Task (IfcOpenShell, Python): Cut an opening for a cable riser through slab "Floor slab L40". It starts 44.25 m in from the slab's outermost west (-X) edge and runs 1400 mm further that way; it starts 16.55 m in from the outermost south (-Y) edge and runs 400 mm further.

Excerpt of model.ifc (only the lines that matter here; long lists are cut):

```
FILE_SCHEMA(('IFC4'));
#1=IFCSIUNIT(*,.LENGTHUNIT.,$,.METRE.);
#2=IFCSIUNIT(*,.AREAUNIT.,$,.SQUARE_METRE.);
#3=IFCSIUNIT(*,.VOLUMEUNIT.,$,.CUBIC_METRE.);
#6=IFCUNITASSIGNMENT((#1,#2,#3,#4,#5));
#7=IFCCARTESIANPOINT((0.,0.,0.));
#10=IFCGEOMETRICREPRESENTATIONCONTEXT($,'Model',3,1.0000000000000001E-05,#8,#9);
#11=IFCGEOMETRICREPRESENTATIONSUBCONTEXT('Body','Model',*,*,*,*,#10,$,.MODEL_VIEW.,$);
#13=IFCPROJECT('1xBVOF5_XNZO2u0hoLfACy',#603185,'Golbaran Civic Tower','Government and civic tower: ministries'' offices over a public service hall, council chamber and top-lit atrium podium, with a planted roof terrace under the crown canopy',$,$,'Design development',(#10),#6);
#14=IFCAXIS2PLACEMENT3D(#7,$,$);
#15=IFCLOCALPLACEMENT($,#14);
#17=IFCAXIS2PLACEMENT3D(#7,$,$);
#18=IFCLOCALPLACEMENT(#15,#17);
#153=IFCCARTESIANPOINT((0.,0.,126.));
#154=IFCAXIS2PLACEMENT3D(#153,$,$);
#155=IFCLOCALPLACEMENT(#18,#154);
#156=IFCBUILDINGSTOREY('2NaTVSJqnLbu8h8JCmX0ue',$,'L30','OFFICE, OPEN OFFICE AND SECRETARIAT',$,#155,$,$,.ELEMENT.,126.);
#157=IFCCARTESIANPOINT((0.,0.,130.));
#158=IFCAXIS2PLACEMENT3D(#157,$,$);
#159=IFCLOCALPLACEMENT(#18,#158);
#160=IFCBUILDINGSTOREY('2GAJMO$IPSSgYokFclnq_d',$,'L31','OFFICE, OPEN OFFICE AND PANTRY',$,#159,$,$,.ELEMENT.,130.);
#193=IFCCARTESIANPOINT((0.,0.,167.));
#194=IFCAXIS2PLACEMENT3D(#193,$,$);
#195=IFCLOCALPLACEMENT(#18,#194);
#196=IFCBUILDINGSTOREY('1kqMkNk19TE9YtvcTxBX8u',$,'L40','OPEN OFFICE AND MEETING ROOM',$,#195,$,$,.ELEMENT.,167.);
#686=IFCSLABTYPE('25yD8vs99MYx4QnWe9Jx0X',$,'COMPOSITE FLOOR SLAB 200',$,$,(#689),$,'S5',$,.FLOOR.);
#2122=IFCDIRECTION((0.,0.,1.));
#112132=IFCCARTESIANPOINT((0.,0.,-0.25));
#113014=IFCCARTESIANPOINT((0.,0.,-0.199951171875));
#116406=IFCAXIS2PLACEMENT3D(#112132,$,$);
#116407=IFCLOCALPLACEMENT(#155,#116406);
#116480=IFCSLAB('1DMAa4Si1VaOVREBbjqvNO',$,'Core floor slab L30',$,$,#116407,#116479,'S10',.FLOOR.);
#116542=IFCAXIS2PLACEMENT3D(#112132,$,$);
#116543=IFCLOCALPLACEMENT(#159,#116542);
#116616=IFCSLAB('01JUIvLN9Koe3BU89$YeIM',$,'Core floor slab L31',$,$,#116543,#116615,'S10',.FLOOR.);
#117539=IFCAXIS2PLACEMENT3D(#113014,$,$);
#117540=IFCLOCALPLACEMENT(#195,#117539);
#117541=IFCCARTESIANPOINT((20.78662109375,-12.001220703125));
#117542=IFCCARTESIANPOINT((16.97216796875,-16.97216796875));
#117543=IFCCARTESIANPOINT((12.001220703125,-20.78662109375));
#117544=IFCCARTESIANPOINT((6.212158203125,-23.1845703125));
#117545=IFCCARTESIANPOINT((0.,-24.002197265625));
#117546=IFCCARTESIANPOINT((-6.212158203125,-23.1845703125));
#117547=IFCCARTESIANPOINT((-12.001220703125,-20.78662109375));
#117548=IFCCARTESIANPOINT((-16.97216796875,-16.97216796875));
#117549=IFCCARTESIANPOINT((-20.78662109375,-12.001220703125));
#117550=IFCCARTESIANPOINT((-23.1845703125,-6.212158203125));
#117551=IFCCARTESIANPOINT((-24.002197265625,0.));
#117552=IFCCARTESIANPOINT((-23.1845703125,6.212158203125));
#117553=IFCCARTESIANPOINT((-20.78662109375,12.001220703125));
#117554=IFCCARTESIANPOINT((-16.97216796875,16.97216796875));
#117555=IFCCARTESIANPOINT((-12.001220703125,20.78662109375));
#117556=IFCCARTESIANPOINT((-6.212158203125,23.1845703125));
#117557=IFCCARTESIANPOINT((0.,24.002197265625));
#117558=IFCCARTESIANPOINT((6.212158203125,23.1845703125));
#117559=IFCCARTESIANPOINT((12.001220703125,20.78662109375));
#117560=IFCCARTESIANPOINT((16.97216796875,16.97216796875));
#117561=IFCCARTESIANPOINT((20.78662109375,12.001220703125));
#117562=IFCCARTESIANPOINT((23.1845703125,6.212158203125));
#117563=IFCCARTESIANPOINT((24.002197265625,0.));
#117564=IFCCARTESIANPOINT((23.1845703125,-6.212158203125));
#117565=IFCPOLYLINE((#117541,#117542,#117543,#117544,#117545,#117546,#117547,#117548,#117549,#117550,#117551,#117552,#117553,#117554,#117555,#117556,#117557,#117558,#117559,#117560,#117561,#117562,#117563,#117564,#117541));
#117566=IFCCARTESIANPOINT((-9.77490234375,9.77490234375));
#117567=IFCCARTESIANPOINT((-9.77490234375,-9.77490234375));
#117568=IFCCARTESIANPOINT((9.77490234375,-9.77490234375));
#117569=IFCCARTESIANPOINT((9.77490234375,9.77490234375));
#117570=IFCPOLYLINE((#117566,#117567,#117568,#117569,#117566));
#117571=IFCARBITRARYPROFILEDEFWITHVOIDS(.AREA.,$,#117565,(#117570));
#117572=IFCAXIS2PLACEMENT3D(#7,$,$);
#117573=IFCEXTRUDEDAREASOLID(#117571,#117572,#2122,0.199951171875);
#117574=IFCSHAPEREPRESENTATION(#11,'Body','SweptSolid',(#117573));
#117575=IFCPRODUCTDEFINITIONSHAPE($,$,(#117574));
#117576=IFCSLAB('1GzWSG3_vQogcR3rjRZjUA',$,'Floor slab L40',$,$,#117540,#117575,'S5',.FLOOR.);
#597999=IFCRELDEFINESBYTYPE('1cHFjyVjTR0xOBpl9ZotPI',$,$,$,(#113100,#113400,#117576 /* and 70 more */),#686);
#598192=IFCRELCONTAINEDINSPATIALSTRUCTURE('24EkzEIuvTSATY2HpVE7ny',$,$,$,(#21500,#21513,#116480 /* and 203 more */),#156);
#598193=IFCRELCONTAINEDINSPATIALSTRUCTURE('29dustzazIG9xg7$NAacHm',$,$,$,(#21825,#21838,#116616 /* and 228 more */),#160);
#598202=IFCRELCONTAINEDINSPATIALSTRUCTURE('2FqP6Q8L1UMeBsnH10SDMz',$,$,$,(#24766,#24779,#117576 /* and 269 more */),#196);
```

```python
import numpy as np
import ifcopenshell
import ifcopenshell.api.feature
import ifcopenshell.api.geometry
import ifcopenshell.api.root
import ifcopenshell.geom
import ifcopenshell.util.placement
import ifcopenshell.util.representation
import ifcopenshell.util.shape
import ifcopenshell.util.unit

model = ifcopenshell.open("model.ifc")
unit_scale = ifcopenshell.util.unit.calculate_unit_scale(model)
settings = ifcopenshell.geom.settings()


def volume(element):
    """Net volume in cubic metres, openings subtracted."""
    shape = ifcopenshell.geom.create_shape(settings, element)
    return ifcopenshell.util.shape.get_volume(shape.geometry)


slab = model.by_guid("1GzWSG3_vQogcR3rjRZjUA")
before = volume(slab)

# Extent in the slab's own axes, in metres. The edges named are its -X and -Y sides.
slab_shape = ifcopenshell.geom.create_shape(settings, slab)
vertices = ifcopenshell.util.shape.get_vertices(slab_shape.geometry)
x_min, y_min, bottom = vertices.min(axis=0)
top = vertices[:, 2].max()

opening = ifcopenshell.api.root.create_entity(model, ifc_class="IfcOpeningElement", name="Cable riser opening", predefined_type="OPENING")
context = ifcopenshell.util.representation.get_context(model, "Model", "Body", "MODEL_VIEW")
width, depth = 1.4, 0.4
outline = [(0.0, 0.0), (width, 0.0), (width, depth), (0.0, depth), (0.0, 0.0)]
# Overshoot both faces by 50 mm so the cut is clean.
shape = ifcopenshell.api.geometry.add_slab_representation(
    model, context=context, depth=top - bottom + 0.1, polyline=outline
)
ifcopenshell.api.geometry.assign_representation(model, product=opening, representation=shape)

matrix = ifcopenshell.util.placement.get_local_placement(slab.ObjectPlacement)
matrix[:, 3] = matrix @ np.append(np.array([x_min + 44.25, y_min + 16.55, bottom - 0.05]) / unit_scale, 1.0)
ifcopenshell.api.geometry.edit_object_placement(model, product=opening, matrix=matrix, is_si=False)
ifcopenshell.api.feature.add_feature(model, feature=opening, element=slab)

after = volume(slab)

print(f"slab volume {before:.3f} -> {after:.3f} m3")

model.write("model-out.ifc")
```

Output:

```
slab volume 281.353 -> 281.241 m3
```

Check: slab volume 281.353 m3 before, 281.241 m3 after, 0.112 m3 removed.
